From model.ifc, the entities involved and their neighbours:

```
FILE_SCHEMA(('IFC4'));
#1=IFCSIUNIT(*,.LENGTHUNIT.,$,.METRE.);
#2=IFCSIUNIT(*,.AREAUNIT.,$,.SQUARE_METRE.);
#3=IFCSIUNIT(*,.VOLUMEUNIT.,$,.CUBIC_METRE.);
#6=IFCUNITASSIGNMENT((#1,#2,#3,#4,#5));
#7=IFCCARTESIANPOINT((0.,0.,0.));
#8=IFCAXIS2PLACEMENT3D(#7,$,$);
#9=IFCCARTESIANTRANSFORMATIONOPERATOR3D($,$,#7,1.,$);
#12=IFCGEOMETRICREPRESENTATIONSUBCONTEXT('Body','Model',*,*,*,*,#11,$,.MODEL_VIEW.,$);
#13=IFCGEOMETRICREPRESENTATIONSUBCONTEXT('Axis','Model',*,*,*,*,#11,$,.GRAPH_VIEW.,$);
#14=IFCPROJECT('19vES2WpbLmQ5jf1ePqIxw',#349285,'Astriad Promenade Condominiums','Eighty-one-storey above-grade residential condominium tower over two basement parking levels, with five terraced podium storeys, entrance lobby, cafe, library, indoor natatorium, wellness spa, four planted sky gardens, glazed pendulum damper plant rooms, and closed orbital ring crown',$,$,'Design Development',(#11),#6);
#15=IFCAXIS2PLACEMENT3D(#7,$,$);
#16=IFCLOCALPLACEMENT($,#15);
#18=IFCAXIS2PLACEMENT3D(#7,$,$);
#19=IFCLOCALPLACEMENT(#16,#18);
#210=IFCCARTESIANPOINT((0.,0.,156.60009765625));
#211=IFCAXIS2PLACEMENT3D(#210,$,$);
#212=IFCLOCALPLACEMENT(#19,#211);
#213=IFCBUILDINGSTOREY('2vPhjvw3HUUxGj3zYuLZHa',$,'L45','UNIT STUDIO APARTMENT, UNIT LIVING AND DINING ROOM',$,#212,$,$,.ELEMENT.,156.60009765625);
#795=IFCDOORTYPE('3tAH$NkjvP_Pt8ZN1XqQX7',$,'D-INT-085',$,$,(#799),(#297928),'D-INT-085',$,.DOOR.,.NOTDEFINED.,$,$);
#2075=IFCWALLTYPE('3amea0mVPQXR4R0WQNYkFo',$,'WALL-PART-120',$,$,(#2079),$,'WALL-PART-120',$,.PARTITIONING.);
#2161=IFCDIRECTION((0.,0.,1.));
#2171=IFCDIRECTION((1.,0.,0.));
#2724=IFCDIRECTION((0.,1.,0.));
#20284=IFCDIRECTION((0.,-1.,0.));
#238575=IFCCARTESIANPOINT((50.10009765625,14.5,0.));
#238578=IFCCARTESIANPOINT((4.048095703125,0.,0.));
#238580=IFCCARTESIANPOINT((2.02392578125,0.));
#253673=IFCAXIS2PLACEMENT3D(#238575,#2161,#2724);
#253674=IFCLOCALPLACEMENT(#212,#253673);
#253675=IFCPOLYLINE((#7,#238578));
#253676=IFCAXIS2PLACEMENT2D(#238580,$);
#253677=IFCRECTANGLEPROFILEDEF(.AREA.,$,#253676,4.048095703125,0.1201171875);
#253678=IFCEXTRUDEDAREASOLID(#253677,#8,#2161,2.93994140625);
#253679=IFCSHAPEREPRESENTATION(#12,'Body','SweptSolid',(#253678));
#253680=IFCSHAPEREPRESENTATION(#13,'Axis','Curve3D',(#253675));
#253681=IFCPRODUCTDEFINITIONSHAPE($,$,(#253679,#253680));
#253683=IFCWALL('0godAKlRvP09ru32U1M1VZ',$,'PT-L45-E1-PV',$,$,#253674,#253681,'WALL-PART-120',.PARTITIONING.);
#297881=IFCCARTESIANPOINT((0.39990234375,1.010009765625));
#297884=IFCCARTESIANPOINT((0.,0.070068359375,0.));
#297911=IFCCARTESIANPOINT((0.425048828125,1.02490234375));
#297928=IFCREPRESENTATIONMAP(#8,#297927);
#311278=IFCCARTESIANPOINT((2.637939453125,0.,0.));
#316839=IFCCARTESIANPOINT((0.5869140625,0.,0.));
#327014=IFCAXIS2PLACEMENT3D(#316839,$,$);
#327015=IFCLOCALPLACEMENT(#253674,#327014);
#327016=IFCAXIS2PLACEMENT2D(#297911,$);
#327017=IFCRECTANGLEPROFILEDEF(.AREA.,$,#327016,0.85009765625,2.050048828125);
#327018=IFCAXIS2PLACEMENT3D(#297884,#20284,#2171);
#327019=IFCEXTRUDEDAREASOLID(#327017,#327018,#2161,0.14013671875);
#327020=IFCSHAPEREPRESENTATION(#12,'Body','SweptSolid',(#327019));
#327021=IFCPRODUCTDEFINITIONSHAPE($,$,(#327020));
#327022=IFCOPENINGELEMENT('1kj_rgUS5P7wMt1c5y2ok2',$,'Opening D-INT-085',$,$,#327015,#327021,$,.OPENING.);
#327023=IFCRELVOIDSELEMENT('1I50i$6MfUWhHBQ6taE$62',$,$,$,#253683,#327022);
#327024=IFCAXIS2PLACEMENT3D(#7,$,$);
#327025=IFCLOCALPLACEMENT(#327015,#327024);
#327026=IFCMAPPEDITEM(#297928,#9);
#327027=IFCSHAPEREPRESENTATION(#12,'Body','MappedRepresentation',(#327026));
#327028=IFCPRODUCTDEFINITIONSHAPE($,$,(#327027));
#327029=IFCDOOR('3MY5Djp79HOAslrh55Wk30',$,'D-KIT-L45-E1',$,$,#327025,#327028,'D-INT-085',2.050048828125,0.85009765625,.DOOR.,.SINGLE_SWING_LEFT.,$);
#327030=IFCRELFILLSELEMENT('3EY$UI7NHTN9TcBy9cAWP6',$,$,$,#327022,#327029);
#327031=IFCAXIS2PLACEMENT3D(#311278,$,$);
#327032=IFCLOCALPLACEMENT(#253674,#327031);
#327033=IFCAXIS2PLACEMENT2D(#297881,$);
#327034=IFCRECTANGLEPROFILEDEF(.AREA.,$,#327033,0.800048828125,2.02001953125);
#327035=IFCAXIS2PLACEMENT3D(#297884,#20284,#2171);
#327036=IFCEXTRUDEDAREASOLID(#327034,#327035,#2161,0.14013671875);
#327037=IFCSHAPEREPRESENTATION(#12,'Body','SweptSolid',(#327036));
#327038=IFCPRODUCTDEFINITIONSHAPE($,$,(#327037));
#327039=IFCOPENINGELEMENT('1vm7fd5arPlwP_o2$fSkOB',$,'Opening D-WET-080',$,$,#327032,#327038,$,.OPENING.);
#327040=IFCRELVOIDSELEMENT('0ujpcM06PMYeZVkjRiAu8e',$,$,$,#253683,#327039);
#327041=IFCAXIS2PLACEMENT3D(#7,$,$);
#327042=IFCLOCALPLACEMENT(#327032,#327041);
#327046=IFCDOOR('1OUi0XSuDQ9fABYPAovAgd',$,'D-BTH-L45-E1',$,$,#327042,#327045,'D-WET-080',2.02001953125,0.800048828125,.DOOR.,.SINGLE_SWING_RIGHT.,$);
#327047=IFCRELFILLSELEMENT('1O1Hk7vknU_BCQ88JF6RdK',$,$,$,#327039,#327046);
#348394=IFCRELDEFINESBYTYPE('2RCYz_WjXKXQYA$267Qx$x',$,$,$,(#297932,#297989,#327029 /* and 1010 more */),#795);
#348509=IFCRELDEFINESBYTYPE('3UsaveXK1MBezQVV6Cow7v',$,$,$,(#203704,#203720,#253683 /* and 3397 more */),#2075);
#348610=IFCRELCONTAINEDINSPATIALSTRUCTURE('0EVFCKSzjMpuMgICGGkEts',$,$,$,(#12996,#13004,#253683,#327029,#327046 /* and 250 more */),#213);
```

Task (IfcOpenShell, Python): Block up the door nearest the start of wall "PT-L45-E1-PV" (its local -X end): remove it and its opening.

```python
import ifcopenshell
import ifcopenshell.api.feature
import ifcopenshell.api.root
import ifcopenshell.geom
import ifcopenshell.util.shape

model = ifcopenshell.open("model.ifc")
settings = ifcopenshell.geom.settings()


def volume(element):
    """Net volume in cubic metres, openings subtracted."""
    shape = ifcopenshell.geom.create_shape(settings, element)
    return ifcopenshell.util.shape.get_volume(shape.geometry)


door = model.by_guid("3MY5Djp79HOAslrh55Wk30")
opening = door.FillsVoids[0].RelatingOpeningElement
wall = opening.VoidsElements[0].RelatingBuildingElement
before = volume(wall)

ifcopenshell.api.root.remove_product(model, product=door)
ifcopenshell.api.feature.remove_feature(model, feature=opening)

after = volume(wall)

print(f"wall volume {before:.3f} -> {after:.3f} m3")

model.write("model-out.ifc")
```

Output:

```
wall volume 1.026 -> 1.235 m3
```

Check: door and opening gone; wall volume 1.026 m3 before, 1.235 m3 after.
